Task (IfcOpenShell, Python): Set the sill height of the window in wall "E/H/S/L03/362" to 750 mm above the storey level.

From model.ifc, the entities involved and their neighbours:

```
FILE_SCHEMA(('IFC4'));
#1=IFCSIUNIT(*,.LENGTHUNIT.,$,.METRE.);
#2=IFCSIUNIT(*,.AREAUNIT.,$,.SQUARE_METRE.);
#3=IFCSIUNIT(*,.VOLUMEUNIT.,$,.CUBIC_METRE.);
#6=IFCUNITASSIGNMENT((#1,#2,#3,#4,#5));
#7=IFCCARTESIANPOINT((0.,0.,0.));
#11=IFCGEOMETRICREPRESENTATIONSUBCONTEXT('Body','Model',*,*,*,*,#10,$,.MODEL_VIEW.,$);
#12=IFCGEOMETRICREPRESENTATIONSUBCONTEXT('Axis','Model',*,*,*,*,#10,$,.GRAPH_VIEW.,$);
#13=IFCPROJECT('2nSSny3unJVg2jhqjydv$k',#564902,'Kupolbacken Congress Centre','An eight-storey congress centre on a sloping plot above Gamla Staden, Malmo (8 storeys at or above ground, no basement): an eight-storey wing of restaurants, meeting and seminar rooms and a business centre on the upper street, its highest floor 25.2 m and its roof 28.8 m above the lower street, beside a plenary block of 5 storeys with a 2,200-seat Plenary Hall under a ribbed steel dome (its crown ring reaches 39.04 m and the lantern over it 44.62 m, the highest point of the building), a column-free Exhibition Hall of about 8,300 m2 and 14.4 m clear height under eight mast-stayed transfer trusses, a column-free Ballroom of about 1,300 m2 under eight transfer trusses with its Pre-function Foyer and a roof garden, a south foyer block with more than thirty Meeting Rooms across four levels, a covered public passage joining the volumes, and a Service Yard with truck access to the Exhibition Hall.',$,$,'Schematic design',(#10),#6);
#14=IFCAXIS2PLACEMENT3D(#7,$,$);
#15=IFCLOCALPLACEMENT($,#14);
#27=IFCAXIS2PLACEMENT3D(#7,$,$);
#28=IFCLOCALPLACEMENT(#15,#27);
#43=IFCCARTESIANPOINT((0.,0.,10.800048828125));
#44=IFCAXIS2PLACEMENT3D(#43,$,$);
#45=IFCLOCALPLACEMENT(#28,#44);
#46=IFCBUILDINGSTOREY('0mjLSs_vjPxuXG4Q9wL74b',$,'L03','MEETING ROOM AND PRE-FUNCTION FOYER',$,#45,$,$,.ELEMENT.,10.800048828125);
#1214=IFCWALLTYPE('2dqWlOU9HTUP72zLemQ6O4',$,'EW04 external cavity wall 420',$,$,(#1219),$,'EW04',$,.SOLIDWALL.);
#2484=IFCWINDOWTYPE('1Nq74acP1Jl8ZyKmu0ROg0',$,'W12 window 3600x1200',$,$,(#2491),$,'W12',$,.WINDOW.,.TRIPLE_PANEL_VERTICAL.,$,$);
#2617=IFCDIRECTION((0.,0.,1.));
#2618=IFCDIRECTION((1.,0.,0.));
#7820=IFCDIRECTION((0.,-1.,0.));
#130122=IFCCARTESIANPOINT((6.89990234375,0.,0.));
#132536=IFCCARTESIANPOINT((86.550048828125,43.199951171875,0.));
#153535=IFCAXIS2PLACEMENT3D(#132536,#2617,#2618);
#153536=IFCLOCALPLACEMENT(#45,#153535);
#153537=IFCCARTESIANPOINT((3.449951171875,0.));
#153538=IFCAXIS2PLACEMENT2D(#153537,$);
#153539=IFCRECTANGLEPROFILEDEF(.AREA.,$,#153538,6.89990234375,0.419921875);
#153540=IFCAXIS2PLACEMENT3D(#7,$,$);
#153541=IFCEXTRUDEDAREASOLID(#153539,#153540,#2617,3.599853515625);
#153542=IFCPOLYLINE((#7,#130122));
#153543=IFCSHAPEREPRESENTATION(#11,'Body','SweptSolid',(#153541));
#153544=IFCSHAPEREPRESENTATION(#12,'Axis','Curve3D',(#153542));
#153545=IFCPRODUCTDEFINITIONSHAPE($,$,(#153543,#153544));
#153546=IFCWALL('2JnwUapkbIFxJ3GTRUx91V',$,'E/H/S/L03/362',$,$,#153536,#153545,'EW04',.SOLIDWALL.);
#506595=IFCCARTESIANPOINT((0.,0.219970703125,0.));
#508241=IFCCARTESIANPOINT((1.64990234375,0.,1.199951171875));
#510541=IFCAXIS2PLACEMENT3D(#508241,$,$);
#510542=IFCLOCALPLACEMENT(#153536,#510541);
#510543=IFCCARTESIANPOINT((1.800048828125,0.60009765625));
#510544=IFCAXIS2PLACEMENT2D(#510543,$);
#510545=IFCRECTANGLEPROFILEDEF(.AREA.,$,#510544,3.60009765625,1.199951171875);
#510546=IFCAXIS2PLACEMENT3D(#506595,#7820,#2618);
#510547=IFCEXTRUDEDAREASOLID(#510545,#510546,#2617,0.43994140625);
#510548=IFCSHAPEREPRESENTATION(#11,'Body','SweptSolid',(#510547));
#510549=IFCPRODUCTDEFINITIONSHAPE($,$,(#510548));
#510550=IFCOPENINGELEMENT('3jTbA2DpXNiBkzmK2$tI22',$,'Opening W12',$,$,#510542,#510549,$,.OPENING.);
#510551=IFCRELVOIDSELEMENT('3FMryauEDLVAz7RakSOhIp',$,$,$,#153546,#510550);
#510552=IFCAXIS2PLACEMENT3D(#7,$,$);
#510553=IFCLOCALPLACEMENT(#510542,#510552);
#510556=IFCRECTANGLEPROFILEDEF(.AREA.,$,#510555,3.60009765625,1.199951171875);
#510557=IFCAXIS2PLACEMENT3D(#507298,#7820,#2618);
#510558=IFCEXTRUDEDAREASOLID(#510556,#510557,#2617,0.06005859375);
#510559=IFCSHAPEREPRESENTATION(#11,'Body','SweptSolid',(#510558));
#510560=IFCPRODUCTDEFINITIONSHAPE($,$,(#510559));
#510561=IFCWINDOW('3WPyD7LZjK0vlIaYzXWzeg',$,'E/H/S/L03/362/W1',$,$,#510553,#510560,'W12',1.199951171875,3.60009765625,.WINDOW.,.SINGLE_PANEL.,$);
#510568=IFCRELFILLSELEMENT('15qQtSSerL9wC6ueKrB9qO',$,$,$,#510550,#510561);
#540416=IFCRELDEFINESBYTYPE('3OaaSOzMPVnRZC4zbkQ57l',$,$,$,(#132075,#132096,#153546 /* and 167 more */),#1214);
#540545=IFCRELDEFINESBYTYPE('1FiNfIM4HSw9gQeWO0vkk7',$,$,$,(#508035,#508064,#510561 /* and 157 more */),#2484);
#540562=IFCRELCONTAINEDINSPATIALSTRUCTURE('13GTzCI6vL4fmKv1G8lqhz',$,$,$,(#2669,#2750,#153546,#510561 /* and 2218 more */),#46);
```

```python
import numpy as np
import ifcopenshell
import ifcopenshell.api.geometry
import ifcopenshell.geom
import ifcopenshell.util.element
import ifcopenshell.util.placement
import ifcopenshell.util.shape
import ifcopenshell.util.unit

model = ifcopenshell.open("model.ifc")
unit_scale = ifcopenshell.util.unit.calculate_unit_scale(model)

window = model.by_guid("3WPyD7LZjK0vlIaYzXWzeg")
opening = window.FillsVoids[0].RelatingOpeningElement
storey = ifcopenshell.util.element.get_container(window, ifc_class="IfcBuildingStorey")
level = ifcopenshell.util.placement.get_local_placement(storey.ObjectPlacement)[2, 3]

# The opening's origin need not be at the sill, so measure its lowest point.
shape = ifcopenshell.geom.create_shape(ifcopenshell.geom.settings(), opening)
bottom = ifcopenshell.util.shape.get_shape_bottom_elevation(shape, shape.geometry) / unit_scale
dz = level + 0.75 / unit_scale - bottom

shift = np.array([0.0, 0.0, dz])
# The window is placed relative to its opening, so it follows when the opening moves.
matrix = ifcopenshell.util.placement.get_local_placement(opening.ObjectPlacement)
matrix[:3, 3] += shift
ifcopenshell.api.geometry.edit_object_placement(
    model, product=opening, matrix=matrix, is_si=False, should_transform_children=True
)

print(f"moved by {dz * unit_scale:+.3f} m")

model.write("model_rev.ifc")
```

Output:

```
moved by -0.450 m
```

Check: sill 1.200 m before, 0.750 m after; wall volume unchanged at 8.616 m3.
